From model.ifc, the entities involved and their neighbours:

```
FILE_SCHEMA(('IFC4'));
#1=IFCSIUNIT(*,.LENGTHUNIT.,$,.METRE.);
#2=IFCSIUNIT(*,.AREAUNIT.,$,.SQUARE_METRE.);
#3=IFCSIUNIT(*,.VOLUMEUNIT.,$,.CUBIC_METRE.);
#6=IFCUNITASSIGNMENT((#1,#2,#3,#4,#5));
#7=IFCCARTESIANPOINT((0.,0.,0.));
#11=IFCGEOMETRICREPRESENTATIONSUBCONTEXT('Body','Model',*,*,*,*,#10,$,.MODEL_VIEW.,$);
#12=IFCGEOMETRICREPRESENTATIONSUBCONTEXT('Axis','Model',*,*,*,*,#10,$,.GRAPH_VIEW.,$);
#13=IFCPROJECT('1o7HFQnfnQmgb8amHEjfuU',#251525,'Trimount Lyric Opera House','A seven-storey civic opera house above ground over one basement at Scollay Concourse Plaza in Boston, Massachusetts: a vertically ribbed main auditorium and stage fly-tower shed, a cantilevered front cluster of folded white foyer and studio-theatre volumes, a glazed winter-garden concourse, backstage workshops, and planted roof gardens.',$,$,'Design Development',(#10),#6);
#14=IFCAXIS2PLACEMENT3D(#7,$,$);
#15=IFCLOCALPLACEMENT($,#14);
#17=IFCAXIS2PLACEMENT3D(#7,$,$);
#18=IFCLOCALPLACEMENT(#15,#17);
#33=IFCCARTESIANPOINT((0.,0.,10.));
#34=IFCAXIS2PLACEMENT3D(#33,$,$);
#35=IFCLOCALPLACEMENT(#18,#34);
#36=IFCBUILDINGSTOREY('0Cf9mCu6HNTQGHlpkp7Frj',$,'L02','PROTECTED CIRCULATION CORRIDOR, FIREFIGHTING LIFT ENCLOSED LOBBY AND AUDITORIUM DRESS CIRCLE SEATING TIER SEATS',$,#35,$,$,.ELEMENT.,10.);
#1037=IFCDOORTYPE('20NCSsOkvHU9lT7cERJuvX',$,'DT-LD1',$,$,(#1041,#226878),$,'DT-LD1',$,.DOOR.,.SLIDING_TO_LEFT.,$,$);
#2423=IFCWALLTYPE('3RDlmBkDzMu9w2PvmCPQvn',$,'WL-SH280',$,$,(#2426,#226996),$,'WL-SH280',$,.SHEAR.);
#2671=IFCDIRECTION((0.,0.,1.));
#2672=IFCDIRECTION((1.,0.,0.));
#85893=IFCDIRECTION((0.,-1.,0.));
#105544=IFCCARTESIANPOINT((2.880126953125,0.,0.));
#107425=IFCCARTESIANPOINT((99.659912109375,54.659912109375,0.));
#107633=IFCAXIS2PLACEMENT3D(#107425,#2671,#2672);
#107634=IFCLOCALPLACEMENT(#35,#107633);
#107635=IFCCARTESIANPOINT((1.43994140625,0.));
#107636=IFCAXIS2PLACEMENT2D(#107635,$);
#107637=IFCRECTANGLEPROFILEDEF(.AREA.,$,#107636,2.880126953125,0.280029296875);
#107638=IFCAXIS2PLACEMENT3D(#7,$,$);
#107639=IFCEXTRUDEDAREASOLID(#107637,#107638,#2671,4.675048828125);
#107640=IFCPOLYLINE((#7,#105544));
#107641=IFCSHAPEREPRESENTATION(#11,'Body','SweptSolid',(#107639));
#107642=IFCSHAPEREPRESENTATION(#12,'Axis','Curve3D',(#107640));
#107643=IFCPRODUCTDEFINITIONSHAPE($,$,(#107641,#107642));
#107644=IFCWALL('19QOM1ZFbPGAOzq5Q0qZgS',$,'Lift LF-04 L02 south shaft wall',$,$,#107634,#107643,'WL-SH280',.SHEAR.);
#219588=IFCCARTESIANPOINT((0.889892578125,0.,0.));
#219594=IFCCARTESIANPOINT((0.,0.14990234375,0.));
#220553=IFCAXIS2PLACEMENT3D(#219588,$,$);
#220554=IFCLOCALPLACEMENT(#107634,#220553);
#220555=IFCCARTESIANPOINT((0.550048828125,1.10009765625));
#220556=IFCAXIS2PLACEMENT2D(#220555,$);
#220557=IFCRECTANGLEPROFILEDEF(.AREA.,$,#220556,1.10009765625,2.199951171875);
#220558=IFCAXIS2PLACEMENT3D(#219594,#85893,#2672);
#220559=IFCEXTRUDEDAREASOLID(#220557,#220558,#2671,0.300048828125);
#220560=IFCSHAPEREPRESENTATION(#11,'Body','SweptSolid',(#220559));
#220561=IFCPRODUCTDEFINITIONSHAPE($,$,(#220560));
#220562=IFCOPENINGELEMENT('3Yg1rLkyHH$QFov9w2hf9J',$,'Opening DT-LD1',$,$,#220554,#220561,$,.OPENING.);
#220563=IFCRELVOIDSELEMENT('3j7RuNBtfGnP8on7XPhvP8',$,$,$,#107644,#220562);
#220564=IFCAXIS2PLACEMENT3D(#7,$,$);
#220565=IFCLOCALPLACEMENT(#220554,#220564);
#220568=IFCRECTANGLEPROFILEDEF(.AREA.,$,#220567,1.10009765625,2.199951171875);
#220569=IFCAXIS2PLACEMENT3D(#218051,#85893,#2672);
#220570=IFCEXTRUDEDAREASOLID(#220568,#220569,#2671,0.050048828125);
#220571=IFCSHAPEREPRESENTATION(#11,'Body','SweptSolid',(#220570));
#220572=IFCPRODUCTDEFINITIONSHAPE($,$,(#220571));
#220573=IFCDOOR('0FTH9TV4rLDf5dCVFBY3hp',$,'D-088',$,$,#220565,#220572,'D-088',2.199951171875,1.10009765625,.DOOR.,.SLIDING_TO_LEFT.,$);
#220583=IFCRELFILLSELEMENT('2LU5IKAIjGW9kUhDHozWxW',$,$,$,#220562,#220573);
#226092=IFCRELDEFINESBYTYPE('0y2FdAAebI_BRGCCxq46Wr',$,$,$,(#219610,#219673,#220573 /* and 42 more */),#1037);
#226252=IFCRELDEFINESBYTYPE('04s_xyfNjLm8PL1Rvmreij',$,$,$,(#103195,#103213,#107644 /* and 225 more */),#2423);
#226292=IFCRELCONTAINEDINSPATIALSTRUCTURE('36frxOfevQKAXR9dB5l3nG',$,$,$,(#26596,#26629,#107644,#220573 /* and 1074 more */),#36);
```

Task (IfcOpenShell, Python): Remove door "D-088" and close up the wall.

```python
import ifcopenshell
import ifcopenshell.api.feature
import ifcopenshell.api.root
import ifcopenshell.geom
import ifcopenshell.util.shape

model = ifcopenshell.open("model.ifc")
settings = ifcopenshell.geom.settings()


def volume(element):
    """Net volume in cubic metres, openings subtracted."""
    shape = ifcopenshell.geom.create_shape(settings, element)
    return ifcopenshell.util.shape.get_volume(shape.geometry)


door = model.by_id(220573)
opening = door.FillsVoids[0].RelatingOpeningElement
wall = opening.VoidsElements[0].RelatingBuildingElement
before = volume(wall)

ifcopenshell.api.root.remove_product(model, product=door)
ifcopenshell.api.feature.remove_feature(model, feature=opening)

after = volume(wall)

print(f"wall volume {before:.3f} -> {after:.3f} m3")

model.write("model_edited.ifc")
```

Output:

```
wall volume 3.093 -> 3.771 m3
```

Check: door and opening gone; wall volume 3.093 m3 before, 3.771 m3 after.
